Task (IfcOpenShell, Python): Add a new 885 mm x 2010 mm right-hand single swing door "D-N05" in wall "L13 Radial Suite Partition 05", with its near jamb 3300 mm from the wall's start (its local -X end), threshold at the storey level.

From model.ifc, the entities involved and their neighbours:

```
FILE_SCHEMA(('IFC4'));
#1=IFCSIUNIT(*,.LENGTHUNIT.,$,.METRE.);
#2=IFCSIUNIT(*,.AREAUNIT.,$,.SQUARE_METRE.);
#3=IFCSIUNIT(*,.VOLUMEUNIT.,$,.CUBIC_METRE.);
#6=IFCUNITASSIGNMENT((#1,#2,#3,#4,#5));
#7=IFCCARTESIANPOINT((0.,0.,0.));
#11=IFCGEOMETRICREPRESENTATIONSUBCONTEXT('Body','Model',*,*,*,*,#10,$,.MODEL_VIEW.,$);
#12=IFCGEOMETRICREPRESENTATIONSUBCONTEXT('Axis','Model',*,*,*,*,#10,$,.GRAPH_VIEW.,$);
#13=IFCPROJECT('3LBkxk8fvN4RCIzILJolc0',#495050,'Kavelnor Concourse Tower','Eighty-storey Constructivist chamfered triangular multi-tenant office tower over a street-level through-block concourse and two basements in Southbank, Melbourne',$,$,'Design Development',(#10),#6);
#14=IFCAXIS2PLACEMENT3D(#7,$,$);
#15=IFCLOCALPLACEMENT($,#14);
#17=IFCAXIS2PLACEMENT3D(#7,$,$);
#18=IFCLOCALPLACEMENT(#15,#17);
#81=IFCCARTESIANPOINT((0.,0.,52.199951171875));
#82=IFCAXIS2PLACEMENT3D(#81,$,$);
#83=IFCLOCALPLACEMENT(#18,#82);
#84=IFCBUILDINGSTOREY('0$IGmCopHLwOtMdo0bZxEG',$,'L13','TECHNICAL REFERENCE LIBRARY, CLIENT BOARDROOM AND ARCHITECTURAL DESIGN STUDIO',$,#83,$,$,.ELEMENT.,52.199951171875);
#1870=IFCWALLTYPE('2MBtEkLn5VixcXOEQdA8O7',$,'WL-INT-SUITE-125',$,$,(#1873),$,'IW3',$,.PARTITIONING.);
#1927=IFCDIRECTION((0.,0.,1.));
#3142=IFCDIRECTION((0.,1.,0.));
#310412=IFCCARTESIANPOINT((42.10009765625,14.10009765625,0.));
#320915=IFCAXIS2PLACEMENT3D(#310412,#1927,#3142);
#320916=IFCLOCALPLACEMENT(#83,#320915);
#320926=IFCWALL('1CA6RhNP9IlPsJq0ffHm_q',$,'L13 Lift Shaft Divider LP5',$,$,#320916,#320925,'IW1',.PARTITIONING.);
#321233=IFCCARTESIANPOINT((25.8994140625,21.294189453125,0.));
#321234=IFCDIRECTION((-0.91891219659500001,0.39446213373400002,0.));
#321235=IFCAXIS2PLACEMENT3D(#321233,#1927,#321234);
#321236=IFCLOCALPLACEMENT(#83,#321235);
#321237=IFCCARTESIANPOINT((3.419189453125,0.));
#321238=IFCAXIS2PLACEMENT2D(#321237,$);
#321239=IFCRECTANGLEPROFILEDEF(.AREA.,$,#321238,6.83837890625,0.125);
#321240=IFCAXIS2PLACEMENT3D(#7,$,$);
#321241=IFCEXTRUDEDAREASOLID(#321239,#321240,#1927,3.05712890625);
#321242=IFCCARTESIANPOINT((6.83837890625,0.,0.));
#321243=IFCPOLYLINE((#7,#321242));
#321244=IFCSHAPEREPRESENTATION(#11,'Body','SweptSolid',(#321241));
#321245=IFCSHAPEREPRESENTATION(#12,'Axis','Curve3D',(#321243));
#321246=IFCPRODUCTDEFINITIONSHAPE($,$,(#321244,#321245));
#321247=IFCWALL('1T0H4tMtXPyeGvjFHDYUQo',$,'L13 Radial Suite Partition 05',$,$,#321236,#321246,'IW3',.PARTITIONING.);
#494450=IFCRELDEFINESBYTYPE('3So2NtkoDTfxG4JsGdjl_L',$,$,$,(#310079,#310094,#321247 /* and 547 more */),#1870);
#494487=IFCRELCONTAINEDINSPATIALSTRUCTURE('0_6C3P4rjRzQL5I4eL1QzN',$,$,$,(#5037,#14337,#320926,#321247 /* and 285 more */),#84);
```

```python
import numpy as np
import ifcopenshell
import ifcopenshell.api.feature
import ifcopenshell.api.geometry
import ifcopenshell.api.root
import ifcopenshell.api.spatial
import ifcopenshell.geom
import ifcopenshell.util.element
import ifcopenshell.util.placement
import ifcopenshell.util.representation
import ifcopenshell.util.shape
import ifcopenshell.util.unit

model = ifcopenshell.open("model.ifc")
unit_scale = ifcopenshell.util.unit.calculate_unit_scale(model)
settings = ifcopenshell.geom.settings()


def volume(element):
    """Net volume in cubic metres, openings subtracted."""
    shape = ifcopenshell.geom.create_shape(settings, element)
    return ifcopenshell.util.shape.get_volume(shape.geometry)


wall = model.by_guid("1T0H4tMtXPyeGvjFHDYUQo")
storey = ifcopenshell.util.element.get_container(wall, ifc_class="IfcBuildingStorey")
context = ifcopenshell.util.representation.get_context(model, "Model", "Body", "MODEL_VIEW")
before = volume(wall)

width, height, from_end, sill = 0.885, 2.01, 3.3, 0.0  # metres

# The wall runs along its own X axis, and the end named is its -X end.
wall_shape = ifcopenshell.geom.create_shape(settings, wall)
x, y, z = ifcopenshell.util.shape.get_vertices(wall_shape.geometry).T
start = x.min() + from_end
face, thickness = float(y.min()), float(y.max() - y.min())
wall_matrix = ifcopenshell.util.placement.get_local_placement(wall.ObjectPlacement)
level = ifcopenshell.util.placement.get_local_placement(storey.ObjectPlacement)[2, 3]


def in_wall(x, y):
    """Placement at x, y metres in the wall's axes, at sill height."""
    matrix = wall_matrix.copy()
    matrix[:, 3] = wall_matrix @ np.array([x / unit_scale, y / unit_scale, 0.0, 1.0])
    matrix[2, 3] = level + sill / unit_scale
    return matrix


# Opening: a box that overshoots both wall faces by 50 mm.
opening = ifcopenshell.api.root.create_entity(model, ifc_class="IfcOpeningElement", predefined_type="OPENING")
box = ifcopenshell.api.geometry.add_wall_representation(
    model, context=context, length=width, height=height, thickness=thickness + 0.1
)
ifcopenshell.api.geometry.assign_representation(model, product=opening, representation=box)
ifcopenshell.api.geometry.edit_object_placement(model, product=opening, matrix=in_wall(start, face - 0.05), is_si=False)
ifcopenshell.api.feature.add_feature(model, feature=opening, element=wall)

door = ifcopenshell.api.root.create_entity(model, ifc_class="IfcDoor", name="D-N05", predefined_type="DOOR")
door.OverallWidth, door.OverallHeight = width / unit_scale, height / unit_scale
door.OperationType = "SINGLE_SWING_RIGHT"
body = ifcopenshell.api.geometry.add_door_representation(
    model,
    context=context,
    overall_width=door.OverallWidth,
    overall_height=door.OverallHeight,
    operation_type="SINGLE_SWING_RIGHT",
    lining_properties={"LiningDepth": thickness / unit_scale, "ThresholdDepth": thickness / unit_scale},
)
ifcopenshell.api.geometry.assign_representation(model, product=door, representation=body)
ifcopenshell.api.spatial.assign_container(model, products=[door], relating_structure=storey)
ifcopenshell.api.feature.add_filling(model, opening=opening, element=door)

# The lining spans the wall, so the door starts at the wall face.
ifcopenshell.api.geometry.edit_object_placement(model, product=door, matrix=in_wall(start, face), is_si=False)

after = volume(wall)

print(f"wall volume {before:.3f} -> {after:.3f} m3")

model.write("model-out.ifc")
```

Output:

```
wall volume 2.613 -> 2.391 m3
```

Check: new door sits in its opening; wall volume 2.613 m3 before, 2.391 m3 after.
